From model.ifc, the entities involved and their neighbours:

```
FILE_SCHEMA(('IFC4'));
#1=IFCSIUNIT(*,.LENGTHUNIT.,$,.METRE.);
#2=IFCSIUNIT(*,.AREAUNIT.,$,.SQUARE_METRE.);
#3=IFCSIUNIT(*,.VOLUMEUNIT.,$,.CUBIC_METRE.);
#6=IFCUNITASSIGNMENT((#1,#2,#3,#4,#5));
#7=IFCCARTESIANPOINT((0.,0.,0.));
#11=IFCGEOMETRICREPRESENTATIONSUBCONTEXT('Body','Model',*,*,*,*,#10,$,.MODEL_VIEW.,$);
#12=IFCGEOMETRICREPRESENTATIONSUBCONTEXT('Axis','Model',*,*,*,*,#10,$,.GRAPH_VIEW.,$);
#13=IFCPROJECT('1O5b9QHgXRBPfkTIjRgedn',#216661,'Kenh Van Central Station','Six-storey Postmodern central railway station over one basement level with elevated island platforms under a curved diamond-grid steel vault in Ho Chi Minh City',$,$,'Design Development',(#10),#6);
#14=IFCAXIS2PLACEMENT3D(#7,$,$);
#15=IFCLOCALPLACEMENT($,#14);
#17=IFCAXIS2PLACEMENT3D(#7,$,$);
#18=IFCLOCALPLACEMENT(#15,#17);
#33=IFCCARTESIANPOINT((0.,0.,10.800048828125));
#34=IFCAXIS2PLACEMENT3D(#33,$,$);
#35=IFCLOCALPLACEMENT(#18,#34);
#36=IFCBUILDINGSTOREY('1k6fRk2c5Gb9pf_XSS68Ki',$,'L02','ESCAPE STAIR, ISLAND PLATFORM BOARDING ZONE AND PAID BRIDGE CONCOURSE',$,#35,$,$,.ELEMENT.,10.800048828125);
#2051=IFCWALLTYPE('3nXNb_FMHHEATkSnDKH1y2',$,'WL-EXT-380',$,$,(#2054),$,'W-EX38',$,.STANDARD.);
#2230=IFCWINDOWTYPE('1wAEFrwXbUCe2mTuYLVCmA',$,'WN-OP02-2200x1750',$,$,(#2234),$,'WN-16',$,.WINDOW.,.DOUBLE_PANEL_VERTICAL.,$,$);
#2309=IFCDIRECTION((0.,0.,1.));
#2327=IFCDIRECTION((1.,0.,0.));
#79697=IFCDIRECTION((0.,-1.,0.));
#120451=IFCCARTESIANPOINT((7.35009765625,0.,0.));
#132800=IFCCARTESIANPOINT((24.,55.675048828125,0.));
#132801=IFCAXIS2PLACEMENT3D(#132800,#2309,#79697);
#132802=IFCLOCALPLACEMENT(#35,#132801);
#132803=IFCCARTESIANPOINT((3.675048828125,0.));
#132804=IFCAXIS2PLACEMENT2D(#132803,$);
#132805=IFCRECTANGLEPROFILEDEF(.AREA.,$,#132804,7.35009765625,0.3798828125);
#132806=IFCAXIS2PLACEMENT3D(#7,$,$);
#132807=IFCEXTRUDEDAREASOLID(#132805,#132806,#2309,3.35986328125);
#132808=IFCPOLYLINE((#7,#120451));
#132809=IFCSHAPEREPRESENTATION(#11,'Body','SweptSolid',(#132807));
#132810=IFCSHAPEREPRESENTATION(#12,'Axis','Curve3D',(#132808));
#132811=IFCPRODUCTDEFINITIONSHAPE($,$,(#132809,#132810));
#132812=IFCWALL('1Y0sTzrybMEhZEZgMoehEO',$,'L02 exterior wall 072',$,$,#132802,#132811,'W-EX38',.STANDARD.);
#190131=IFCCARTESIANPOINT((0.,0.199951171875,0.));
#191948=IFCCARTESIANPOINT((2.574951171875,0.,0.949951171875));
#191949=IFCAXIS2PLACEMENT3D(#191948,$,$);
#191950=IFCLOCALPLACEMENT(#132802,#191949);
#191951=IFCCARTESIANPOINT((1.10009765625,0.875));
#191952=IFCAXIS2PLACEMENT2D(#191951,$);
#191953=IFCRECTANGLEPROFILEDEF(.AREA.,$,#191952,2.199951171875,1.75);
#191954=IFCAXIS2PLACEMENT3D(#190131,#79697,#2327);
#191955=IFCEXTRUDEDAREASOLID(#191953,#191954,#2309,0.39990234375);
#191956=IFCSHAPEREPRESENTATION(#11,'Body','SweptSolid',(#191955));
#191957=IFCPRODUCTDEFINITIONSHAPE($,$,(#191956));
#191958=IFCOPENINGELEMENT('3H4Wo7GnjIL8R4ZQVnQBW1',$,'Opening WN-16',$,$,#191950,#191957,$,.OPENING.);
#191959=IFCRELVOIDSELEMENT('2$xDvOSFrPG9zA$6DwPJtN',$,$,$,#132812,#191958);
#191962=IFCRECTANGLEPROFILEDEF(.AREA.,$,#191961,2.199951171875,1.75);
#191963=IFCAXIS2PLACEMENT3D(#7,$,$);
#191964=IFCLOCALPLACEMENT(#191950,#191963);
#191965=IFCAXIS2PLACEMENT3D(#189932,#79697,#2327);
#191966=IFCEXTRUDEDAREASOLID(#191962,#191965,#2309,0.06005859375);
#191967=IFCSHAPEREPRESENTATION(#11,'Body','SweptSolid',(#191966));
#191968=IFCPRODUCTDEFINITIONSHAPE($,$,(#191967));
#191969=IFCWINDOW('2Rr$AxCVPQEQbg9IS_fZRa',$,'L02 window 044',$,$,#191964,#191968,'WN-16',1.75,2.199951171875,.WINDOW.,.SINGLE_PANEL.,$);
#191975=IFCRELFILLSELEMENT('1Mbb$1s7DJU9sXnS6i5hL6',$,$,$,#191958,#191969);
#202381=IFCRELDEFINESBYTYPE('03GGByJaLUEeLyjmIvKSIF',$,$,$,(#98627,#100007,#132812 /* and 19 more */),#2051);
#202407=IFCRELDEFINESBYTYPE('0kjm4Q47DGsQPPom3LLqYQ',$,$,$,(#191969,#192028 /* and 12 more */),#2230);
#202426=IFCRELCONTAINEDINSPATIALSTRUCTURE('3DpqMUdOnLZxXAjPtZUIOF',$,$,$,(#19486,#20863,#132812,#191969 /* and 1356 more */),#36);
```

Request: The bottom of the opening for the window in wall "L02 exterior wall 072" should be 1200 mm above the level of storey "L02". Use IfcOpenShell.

```python
import numpy as np
import ifcopenshell
import ifcopenshell.api.geometry
import ifcopenshell.geom
import ifcopenshell.util.element
import ifcopenshell.util.placement
import ifcopenshell.util.shape
import ifcopenshell.util.unit

model = ifcopenshell.open("model.ifc")
unit_scale = ifcopenshell.util.unit.calculate_unit_scale(model)

window = model.by_id(191969)
opening = window.FillsVoids[0].RelatingOpeningElement
storey = ifcopenshell.util.element.get_container(window, ifc_class="IfcBuildingStorey")
level = ifcopenshell.util.placement.get_local_placement(storey.ObjectPlacement)[2, 3]

# The opening's origin need not be at the sill, so measure its lowest point.
shape = ifcopenshell.geom.create_shape(ifcopenshell.geom.settings(), opening)
bottom = ifcopenshell.util.shape.get_shape_bottom_elevation(shape, shape.geometry) / unit_scale
dz = level + 1.2 / unit_scale - bottom

shift = np.array([0.0, 0.0, dz])
# The window is placed relative to its opening, so it follows when the opening moves.
matrix = ifcopenshell.util.placement.get_local_placement(opening.ObjectPlacement)
matrix[:3, 3] += shift
ifcopenshell.api.geometry.edit_object_placement(
    model, product=opening, matrix=matrix, is_si=False, should_transform_children=True
)

print(f"moved by {dz * unit_scale:+.3f} m")

model.write("model_edited.ifc")
```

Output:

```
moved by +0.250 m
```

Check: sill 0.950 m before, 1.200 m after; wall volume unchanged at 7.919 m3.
